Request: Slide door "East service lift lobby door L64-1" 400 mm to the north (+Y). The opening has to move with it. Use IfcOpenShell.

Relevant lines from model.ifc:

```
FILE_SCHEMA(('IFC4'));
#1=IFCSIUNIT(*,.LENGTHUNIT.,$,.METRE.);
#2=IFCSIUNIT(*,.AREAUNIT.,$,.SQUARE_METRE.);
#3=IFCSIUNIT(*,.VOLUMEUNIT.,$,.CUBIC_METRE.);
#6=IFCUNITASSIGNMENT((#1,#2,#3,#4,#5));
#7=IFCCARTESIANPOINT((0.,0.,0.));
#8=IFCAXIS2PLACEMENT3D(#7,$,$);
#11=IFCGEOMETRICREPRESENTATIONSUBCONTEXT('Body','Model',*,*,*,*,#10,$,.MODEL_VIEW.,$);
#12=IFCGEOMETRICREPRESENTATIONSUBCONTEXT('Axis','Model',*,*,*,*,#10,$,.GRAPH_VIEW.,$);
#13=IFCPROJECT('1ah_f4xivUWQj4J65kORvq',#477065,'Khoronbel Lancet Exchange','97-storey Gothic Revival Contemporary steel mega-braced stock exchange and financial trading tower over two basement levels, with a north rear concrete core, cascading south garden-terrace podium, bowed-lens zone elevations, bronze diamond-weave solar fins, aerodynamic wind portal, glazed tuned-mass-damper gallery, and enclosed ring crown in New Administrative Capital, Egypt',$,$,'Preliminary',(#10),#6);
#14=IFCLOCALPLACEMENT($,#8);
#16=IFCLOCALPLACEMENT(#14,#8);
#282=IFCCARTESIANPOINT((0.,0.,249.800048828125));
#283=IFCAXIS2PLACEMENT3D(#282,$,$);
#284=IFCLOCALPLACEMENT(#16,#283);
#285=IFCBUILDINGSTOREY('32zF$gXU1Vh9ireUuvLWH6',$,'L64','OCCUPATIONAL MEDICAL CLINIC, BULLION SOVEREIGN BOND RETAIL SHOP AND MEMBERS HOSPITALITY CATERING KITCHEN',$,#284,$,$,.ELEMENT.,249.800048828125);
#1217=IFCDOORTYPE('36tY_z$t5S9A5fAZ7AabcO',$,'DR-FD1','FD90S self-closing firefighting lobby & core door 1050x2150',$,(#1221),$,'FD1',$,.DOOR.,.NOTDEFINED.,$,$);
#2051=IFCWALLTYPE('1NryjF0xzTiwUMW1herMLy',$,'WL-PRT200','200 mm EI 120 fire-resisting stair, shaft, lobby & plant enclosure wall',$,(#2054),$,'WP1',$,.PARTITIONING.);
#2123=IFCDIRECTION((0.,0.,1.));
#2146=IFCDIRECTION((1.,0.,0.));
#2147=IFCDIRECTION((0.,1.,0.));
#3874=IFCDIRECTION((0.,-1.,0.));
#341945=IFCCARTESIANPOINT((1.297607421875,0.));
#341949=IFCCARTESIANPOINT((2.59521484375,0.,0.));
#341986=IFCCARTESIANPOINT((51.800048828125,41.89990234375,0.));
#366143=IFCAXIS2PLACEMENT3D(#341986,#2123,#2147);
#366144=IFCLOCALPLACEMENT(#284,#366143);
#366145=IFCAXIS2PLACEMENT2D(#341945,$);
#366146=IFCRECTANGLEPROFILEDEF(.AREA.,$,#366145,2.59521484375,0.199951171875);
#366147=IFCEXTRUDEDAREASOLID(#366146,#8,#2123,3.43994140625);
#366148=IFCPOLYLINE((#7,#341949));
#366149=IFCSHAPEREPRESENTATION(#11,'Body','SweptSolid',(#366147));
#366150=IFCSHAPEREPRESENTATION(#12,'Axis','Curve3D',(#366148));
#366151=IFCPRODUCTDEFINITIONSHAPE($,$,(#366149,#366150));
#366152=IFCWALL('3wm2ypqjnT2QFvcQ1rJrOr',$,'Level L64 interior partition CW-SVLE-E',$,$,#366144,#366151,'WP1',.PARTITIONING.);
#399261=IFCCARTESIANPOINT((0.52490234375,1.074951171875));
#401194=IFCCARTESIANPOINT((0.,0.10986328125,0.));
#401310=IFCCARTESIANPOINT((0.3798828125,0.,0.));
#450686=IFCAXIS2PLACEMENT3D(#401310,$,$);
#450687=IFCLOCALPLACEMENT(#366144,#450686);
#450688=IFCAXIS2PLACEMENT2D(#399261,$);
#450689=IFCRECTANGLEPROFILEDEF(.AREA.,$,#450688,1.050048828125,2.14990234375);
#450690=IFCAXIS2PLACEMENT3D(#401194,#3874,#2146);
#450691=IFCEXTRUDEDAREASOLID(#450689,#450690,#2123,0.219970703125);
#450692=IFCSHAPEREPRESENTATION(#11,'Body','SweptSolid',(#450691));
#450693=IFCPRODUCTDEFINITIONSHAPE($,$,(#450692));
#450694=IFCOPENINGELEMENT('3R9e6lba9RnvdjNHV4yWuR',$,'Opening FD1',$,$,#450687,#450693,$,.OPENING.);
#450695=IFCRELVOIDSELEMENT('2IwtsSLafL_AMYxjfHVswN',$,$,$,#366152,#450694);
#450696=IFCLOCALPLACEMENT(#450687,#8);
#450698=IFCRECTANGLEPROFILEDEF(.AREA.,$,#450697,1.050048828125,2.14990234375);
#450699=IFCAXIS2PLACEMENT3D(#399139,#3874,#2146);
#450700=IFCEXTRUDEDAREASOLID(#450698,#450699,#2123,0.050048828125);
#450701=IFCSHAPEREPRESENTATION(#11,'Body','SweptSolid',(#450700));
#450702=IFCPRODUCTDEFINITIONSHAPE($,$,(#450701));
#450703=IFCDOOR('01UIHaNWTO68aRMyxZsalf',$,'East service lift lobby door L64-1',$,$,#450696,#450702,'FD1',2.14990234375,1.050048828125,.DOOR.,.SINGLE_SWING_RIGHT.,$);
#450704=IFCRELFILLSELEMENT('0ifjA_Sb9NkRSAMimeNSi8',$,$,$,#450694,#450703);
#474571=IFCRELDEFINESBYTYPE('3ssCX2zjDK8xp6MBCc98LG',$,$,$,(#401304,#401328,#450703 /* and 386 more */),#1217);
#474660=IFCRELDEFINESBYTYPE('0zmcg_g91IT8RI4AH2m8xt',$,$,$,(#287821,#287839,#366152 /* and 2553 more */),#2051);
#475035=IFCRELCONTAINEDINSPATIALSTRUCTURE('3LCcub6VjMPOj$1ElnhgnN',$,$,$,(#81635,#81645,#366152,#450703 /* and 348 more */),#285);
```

```python
import ifcopenshell
import ifcopenshell.api.geometry
import ifcopenshell.util.placement

model = ifcopenshell.open("model.ifc")

door = model.by_guid("01UIHaNWTO68aRMyxZsalf")
opening = door.FillsVoids[0].RelatingOpeningElement
wall = opening.VoidsElements[0].RelatingBuildingElement

wall_matrix = ifcopenshell.util.placement.get_local_placement(wall.ObjectPlacement)
shift = wall_matrix[:3, 0] * 0.4
before = ifcopenshell.util.placement.get_local_placement(door.ObjectPlacement)[:3, 3].copy()

# The door is placed relative to its opening, so it follows when the opening moves.
matrix = ifcopenshell.util.placement.get_local_placement(opening.ObjectPlacement)
matrix[:3, 3] += shift
ifcopenshell.api.geometry.edit_object_placement(
    model, product=opening, matrix=matrix, is_si=False, should_transform_children=True
)

after = ifcopenshell.util.placement.get_local_placement(door.ObjectPlacement)[:3, 3]
print("door moved by", (after - before).round(3) + 0.0)

model.write("model_v2.ifc")
```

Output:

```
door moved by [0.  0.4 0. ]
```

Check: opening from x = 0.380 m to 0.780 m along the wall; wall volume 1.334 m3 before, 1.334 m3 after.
